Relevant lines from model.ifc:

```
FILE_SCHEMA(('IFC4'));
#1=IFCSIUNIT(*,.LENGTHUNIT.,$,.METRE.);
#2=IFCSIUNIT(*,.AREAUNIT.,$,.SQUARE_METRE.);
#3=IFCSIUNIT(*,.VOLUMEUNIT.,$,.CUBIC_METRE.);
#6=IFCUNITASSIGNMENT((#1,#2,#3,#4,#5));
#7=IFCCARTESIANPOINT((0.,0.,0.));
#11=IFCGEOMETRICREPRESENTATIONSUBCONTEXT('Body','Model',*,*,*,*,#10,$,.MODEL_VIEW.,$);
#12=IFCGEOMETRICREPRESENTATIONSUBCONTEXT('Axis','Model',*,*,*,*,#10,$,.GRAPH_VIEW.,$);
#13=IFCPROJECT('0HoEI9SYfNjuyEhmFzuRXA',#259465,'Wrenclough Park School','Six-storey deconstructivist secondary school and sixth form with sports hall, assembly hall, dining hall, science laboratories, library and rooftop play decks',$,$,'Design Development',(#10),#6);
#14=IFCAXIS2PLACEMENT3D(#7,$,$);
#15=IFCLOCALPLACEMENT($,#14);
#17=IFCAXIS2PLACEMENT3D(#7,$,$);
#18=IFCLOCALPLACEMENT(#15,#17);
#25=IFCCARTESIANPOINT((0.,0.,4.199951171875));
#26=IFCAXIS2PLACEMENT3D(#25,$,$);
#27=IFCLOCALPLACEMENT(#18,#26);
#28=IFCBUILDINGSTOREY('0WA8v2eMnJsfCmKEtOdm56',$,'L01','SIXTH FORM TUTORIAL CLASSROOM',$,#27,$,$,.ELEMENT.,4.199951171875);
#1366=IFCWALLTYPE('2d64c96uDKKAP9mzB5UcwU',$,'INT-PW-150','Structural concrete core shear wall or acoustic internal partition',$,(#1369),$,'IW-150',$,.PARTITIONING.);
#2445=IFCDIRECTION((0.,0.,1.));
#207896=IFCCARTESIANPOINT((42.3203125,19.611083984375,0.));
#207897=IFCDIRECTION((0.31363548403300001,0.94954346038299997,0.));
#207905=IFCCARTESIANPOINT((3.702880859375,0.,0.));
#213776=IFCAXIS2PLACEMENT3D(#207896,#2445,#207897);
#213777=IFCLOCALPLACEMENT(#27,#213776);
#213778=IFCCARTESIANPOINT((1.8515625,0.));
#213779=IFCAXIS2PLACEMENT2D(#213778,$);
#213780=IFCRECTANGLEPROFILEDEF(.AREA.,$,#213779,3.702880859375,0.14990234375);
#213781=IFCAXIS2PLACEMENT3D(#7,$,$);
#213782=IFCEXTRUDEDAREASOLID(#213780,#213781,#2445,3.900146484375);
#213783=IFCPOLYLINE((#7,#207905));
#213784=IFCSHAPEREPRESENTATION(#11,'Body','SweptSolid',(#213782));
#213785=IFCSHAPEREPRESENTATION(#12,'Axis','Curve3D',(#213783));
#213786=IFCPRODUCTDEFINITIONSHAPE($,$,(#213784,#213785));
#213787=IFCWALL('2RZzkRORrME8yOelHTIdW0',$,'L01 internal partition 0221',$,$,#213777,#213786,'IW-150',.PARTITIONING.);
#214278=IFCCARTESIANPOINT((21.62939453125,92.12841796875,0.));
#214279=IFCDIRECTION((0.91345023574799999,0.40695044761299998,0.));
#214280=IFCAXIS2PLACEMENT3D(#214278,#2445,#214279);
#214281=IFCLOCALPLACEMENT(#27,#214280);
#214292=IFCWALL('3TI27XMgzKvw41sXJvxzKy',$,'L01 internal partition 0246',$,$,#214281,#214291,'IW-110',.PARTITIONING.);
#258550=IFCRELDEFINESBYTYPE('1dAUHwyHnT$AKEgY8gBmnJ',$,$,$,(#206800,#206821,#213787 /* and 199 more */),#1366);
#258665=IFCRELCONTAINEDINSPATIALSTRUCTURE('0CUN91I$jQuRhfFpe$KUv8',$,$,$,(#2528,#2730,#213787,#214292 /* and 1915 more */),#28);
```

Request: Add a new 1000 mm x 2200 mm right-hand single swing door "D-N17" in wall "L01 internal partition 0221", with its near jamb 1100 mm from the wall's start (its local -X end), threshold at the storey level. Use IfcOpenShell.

```python
import numpy as np
import ifcopenshell
import ifcopenshell.api.feature
import ifcopenshell.api.geometry
import ifcopenshell.api.root
import ifcopenshell.api.spatial
import ifcopenshell.geom
import ifcopenshell.util.element
import ifcopenshell.util.placement
import ifcopenshell.util.representation
import ifcopenshell.util.shape
import ifcopenshell.util.unit

model = ifcopenshell.open("model.ifc")
unit_scale = ifcopenshell.util.unit.calculate_unit_scale(model)
settings = ifcopenshell.geom.settings()


def volume(element):
    """Net volume in cubic metres, openings subtracted."""
    shape = ifcopenshell.geom.create_shape(settings, element)
    return ifcopenshell.util.shape.get_volume(shape.geometry)


wall = model.by_guid("2RZzkRORrME8yOelHTIdW0")
storey = ifcopenshell.util.element.get_container(wall, ifc_class="IfcBuildingStorey")
context = ifcopenshell.util.representation.get_context(model, "Model", "Body", "MODEL_VIEW")
before = volume(wall)

width, height, from_end, sill = 1, 2.2, 1.1, 0.0  # metres

# The wall runs along its own X axis, and the end named is its -X end.
wall_shape = ifcopenshell.geom.create_shape(settings, wall)
x, y, z = ifcopenshell.util.shape.get_vertices(wall_shape.geometry).T
start = x.min() + from_end
face, thickness = float(y.min()), float(y.max() - y.min())
wall_matrix = ifcopenshell.util.placement.get_local_placement(wall.ObjectPlacement)
level = ifcopenshell.util.placement.get_local_placement(storey.ObjectPlacement)[2, 3]


def in_wall(x, y):
    """Placement at x, y metres in the wall's axes, at sill height."""
    matrix = wall_matrix.copy()
    matrix[:, 3] = wall_matrix @ np.array([x / unit_scale, y / unit_scale, 0.0, 1.0])
    matrix[2, 3] = level + sill / unit_scale
    return matrix


# Opening: a box that overshoots both wall faces by 50 mm.
opening = ifcopenshell.api.root.create_entity(model, ifc_class="IfcOpeningElement", predefined_type="OPENING")
box = ifcopenshell.api.geometry.add_wall_representation(
    model, context=context, length=width, height=height, thickness=thickness + 0.1
)
ifcopenshell.api.geometry.assign_representation(model, product=opening, representation=box)
ifcopenshell.api.geometry.edit_object_placement(model, product=opening, matrix=in_wall(start, face - 0.05), is_si=False)
ifcopenshell.api.feature.add_feature(model, feature=opening, element=wall)

door = ifcopenshell.api.root.create_entity(model, ifc_class="IfcDoor", name="D-N17", predefined_type="DOOR")
door.OverallWidth, door.OverallHeight = width / unit_scale, height / unit_scale
door.OperationType = "SINGLE_SWING_RIGHT"
body = ifcopenshell.api.geometry.add_door_representation(
    model,
    context=context,
    overall_width=door.OverallWidth,
    overall_height=door.OverallHeight,
    operation_type="SINGLE_SWING_RIGHT",
    lining_properties={"LiningDepth": thickness / unit_scale, "ThresholdDepth": thickness / unit_scale},
)
ifcopenshell.api.geometry.assign_representation(model, product=door, representation=body)
ifcopenshell.api.spatial.assign_container(model, products=[door], relating_structure=storey)
ifcopenshell.api.feature.add_filling(model, opening=opening, element=door)

# The lining spans the wall, so the door starts at the wall face.
ifcopenshell.api.geometry.edit_object_placement(model, product=door, matrix=in_wall(start, face), is_si=False)

after = volume(wall)

print(f"wall volume {before:.3f} -> {after:.3f} m3")

model.write("model_edited.ifc")
```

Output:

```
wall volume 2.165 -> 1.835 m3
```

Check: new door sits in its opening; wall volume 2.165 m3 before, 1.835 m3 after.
